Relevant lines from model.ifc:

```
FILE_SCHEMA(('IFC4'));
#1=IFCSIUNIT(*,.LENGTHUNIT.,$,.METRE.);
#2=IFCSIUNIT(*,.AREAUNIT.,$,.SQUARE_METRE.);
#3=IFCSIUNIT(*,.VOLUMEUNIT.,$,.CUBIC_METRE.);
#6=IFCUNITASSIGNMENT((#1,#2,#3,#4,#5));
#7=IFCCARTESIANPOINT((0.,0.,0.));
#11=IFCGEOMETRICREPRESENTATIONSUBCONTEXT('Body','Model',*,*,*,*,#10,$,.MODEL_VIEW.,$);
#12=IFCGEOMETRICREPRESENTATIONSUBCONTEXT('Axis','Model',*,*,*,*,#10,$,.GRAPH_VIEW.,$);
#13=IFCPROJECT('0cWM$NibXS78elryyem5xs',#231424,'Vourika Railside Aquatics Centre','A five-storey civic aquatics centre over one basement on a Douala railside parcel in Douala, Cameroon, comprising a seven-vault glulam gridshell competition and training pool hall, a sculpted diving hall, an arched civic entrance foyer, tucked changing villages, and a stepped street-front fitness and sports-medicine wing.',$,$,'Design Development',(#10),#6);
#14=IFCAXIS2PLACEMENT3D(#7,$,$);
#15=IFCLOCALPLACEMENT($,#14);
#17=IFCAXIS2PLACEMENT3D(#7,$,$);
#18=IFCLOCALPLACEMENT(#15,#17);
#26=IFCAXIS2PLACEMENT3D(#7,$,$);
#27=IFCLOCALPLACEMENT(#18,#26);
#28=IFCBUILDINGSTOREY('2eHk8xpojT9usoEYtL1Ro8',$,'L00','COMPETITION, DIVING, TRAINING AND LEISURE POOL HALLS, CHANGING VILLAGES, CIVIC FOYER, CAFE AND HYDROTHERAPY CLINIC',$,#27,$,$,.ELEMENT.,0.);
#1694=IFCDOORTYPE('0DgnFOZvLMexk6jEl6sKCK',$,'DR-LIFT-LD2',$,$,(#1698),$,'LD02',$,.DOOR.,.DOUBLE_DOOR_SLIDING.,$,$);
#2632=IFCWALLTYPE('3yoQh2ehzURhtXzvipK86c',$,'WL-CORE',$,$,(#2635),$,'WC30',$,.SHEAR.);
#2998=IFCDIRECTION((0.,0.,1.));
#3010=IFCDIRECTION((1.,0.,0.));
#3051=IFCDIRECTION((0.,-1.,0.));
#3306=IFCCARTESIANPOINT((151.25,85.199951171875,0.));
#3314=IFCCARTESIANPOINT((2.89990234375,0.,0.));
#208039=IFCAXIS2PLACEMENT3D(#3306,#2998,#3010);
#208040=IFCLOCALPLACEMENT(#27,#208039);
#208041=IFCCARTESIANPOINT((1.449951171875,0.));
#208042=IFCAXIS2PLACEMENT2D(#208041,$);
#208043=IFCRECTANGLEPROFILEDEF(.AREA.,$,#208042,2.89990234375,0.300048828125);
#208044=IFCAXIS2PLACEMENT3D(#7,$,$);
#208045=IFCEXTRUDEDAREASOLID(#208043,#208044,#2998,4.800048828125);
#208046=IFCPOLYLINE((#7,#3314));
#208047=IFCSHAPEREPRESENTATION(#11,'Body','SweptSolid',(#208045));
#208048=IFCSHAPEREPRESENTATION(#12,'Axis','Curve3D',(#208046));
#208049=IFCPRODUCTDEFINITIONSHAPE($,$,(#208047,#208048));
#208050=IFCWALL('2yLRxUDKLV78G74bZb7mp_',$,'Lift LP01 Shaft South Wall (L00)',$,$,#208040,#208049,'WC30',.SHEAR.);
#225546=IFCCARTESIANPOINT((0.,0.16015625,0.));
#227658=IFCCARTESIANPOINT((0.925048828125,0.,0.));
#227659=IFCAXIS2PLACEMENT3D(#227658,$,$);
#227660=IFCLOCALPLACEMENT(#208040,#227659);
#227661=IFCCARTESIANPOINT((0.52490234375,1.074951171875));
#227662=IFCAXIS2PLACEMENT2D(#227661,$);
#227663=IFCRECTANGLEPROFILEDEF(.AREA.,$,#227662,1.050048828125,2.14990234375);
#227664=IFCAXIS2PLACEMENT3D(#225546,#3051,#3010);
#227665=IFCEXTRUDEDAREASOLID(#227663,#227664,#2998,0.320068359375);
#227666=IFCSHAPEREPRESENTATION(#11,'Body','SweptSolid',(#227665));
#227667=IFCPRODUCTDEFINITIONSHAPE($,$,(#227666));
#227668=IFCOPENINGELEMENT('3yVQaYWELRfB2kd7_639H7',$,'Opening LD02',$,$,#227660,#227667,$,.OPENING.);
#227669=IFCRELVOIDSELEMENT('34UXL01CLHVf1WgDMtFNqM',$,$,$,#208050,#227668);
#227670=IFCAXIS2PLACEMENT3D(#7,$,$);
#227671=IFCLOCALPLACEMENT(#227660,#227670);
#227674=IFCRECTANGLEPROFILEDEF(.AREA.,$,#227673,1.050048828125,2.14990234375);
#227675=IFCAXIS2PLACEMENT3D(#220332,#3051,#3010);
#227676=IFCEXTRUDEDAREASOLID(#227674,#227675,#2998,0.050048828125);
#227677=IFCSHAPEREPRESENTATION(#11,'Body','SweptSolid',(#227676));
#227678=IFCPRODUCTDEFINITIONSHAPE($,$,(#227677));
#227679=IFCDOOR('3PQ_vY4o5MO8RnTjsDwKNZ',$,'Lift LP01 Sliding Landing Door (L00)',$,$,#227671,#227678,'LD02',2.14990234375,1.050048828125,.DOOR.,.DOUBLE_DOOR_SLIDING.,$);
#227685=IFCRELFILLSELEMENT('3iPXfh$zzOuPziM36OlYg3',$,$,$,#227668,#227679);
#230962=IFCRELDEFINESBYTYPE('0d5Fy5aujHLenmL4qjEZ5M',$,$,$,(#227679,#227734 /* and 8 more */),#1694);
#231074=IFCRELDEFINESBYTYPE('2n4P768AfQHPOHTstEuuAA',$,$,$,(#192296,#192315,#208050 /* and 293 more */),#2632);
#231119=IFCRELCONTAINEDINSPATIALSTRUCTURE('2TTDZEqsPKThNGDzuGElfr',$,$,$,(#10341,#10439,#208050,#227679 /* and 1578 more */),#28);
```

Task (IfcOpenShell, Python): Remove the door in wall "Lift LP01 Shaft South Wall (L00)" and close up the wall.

```python
import ifcopenshell
import ifcopenshell.api.feature
import ifcopenshell.api.root
import ifcopenshell.geom
import ifcopenshell.util.shape

model = ifcopenshell.open("model.ifc")
settings = ifcopenshell.geom.settings()


def volume(element):
    """Net volume in cubic metres, openings subtracted."""
    shape = ifcopenshell.geom.create_shape(settings, element)
    return ifcopenshell.util.shape.get_volume(shape.geometry)


door = model.by_guid("3PQ_vY4o5MO8RnTjsDwKNZ")
opening = door.FillsVoids[0].RelatingOpeningElement
wall = opening.VoidsElements[0].RelatingBuildingElement
before = volume(wall)

ifcopenshell.api.root.remove_product(model, product=door)
ifcopenshell.api.feature.remove_feature(model, feature=opening)

after = volume(wall)

print(f"wall volume {before:.3f} -> {after:.3f} m3")

model.write("model_edited.ifc")
```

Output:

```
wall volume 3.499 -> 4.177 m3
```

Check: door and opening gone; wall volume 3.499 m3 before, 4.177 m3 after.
